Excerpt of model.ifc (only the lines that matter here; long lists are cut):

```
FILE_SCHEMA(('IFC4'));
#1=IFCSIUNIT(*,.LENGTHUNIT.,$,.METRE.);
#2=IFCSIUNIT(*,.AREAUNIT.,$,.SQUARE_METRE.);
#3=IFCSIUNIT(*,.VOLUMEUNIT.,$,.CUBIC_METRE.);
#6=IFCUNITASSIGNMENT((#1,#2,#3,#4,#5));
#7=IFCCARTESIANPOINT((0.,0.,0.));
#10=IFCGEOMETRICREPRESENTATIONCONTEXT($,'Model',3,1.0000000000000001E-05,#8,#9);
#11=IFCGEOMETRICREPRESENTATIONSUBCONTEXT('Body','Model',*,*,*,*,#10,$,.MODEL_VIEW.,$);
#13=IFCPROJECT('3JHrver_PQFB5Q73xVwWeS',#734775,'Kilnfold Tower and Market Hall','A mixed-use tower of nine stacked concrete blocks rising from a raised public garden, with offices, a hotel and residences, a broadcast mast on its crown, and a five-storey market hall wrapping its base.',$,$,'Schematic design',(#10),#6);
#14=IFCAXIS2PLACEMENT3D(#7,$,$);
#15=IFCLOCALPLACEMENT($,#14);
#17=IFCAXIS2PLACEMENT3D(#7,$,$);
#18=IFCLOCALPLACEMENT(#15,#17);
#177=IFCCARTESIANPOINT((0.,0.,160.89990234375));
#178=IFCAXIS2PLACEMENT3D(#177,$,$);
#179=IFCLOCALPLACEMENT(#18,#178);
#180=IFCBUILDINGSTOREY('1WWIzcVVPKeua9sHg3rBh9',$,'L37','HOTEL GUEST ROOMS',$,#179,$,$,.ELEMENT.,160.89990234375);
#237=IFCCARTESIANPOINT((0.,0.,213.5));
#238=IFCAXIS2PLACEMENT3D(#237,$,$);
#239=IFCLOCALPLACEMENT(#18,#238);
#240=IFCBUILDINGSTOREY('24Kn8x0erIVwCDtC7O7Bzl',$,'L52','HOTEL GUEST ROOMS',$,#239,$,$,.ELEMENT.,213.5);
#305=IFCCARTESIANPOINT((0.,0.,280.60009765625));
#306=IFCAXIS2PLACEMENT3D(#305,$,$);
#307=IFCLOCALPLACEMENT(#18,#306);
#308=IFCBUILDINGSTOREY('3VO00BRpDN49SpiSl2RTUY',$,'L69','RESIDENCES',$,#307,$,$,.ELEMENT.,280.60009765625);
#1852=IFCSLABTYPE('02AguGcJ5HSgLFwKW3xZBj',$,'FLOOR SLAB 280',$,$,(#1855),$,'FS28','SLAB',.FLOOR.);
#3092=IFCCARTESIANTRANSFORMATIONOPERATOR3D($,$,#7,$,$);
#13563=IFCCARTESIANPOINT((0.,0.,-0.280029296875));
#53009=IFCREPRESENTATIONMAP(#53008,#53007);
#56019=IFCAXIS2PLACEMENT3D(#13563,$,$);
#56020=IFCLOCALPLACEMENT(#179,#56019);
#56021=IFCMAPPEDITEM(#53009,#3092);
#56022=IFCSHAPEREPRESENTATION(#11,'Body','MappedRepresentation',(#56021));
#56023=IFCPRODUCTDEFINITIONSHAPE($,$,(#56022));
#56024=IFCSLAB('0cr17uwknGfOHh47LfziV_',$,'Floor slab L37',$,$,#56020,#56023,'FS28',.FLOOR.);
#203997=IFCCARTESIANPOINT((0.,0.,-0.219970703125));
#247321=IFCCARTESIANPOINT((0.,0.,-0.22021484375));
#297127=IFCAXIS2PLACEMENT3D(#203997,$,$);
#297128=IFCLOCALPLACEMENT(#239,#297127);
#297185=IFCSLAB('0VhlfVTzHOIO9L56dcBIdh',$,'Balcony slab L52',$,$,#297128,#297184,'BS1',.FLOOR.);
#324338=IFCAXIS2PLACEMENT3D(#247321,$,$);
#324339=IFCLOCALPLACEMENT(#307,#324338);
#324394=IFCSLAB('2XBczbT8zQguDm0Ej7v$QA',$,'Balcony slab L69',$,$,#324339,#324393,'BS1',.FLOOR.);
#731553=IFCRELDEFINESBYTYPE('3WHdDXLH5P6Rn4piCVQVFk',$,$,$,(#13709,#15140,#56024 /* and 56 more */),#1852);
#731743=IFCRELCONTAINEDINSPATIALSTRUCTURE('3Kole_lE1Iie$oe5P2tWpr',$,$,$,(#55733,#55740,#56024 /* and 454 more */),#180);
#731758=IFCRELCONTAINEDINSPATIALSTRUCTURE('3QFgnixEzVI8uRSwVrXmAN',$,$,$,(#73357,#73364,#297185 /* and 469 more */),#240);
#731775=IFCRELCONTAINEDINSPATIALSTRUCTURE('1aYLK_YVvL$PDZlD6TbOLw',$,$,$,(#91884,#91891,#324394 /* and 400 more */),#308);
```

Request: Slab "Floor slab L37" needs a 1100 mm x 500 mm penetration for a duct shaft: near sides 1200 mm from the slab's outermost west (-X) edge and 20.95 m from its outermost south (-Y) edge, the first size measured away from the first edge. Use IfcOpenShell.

```python
import numpy as np
import ifcopenshell
import ifcopenshell.api.feature
import ifcopenshell.api.geometry
import ifcopenshell.api.root
import ifcopenshell.geom
import ifcopenshell.util.placement
import ifcopenshell.util.representation
import ifcopenshell.util.shape
import ifcopenshell.util.unit

model = ifcopenshell.open("model.ifc")
unit_scale = ifcopenshell.util.unit.calculate_unit_scale(model)
settings = ifcopenshell.geom.settings()


def volume(element):
    """Net volume in cubic metres, openings subtracted."""
    shape = ifcopenshell.geom.create_shape(settings, element)
    return ifcopenshell.util.shape.get_volume(shape.geometry)


slab = model.by_guid("0cr17uwknGfOHh47LfziV_")
before = volume(slab)

# Extent in the slab's own axes, in metres. The edges named are its -X and -Y sides.
slab_shape = ifcopenshell.geom.create_shape(settings, slab)
vertices = ifcopenshell.util.shape.get_vertices(slab_shape.geometry)
x_min, y_min, bottom = vertices.min(axis=0)
top = vertices[:, 2].max()

opening = ifcopenshell.api.root.create_entity(model, ifc_class="IfcOpeningElement", name="Duct shaft opening", predefined_type="OPENING")
context = ifcopenshell.util.representation.get_context(model, "Model", "Body", "MODEL_VIEW")
width, depth = 1.1, 0.5
outline = [(0.0, 0.0), (width, 0.0), (width, depth), (0.0, depth), (0.0, 0.0)]
# Overshoot both faces by 50 mm so the cut is clean.
shape = ifcopenshell.api.geometry.add_slab_representation(
    model, context=context, depth=top - bottom + 0.1, polyline=outline
)
ifcopenshell.api.geometry.assign_representation(model, product=opening, representation=shape)

matrix = ifcopenshell.util.placement.get_local_placement(slab.ObjectPlacement)
matrix[:, 3] = matrix @ np.append(np.array([x_min + 1.2, y_min + 20.95, bottom - 0.05]) / unit_scale, 1.0)
ifcopenshell.api.geometry.edit_object_placement(model, product=opening, matrix=matrix, is_si=False)
ifcopenshell.api.feature.add_feature(model, feature=opening, element=slab)

after = volume(slab)

print(f"slab volume {before:.3f} -> {after:.3f} m3")

model.write("model_updated.ifc")
```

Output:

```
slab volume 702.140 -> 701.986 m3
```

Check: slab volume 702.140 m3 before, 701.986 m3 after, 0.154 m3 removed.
